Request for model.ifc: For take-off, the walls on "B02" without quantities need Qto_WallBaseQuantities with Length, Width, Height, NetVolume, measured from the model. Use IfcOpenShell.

First a look at what the model holds.

```python
import ifcopenshell
import ifcopenshell.util.element
import ifcopenshell.util.unit

model = ifcopenshell.open("model.ifc")
print(model.schema)
for unit_type in ("LENGTHUNIT", "AREAUNIT", "VOLUMEUNIT"):
    print(unit_type, ifcopenshell.util.unit.calculate_unit_scale(model, unit_type))
storey = next(s for s in model.by_type("IfcBuildingStorey") if s.Name == "B02")
walls = [e for e in ifcopenshell.util.element.get_decomposition(storey) if e.is_a("IfcWall")]
for e in sorted(walls, key=lambda e: e.id()):
    print(e.id(), e.is_a(), e.Name, list(ifcopenshell.util.element.get_psets(e, qtos_only=True)), sep=" | ")
```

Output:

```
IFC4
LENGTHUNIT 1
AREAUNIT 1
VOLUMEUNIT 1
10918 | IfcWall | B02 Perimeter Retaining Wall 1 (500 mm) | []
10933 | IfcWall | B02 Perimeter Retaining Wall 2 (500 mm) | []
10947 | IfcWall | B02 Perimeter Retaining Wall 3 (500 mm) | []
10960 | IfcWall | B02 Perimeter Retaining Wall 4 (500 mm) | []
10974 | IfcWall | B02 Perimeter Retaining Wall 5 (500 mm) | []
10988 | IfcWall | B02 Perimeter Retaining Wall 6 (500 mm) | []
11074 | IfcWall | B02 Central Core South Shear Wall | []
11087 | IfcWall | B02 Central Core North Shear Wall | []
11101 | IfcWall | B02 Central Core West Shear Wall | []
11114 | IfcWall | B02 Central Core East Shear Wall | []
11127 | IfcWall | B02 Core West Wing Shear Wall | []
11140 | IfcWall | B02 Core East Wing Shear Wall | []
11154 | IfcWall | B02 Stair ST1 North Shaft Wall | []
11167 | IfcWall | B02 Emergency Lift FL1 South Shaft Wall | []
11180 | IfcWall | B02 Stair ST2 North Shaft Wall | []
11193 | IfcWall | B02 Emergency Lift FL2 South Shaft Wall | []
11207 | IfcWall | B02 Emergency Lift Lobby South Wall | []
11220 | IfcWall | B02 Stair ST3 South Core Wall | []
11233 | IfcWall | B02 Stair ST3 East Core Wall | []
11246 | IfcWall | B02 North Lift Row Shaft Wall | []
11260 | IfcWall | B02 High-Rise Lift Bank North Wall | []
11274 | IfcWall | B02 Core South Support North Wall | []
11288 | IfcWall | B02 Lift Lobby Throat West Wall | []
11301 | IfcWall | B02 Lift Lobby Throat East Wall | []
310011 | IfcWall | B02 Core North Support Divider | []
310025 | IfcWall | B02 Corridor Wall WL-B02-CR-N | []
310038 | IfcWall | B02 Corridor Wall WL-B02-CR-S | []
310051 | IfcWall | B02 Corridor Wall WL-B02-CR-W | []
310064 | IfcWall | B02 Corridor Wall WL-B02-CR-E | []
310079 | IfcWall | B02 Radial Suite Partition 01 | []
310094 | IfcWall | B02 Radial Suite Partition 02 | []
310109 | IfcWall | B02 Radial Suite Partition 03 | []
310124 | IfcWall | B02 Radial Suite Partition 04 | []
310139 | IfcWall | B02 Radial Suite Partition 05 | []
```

```python
import ifcopenshell
import ifcopenshell.api.pset
import ifcopenshell.geom
import ifcopenshell.util.element
import ifcopenshell.util.shape
import ifcopenshell.util.unit

model = ifcopenshell.open("model.ifc")
unit_scale = ifcopenshell.util.unit.calculate_unit_scale(model)
volume_scale = ifcopenshell.util.unit.calculate_unit_scale(model, "VOLUMEUNIT")
settings = ifcopenshell.geom.settings()

storey = next(s for s in model.by_type("IfcBuildingStorey") if s.Name == "B02")
walls = [e for e in ifcopenshell.util.element.get_decomposition(storey) if e.is_a("IfcWall")]

for e in sorted(walls, key=lambda e: e.id()):
    if ifcopenshell.util.element.get_psets(e, qtos_only=True, should_inherit=False):
        continue
    # Geometry comes back in metres, in the element's own axes.
    shape = ifcopenshell.geom.create_shape(settings, e)
    values = {
        "Length": ifcopenshell.util.shape.get_x(shape.geometry) / unit_scale,
        "Width": ifcopenshell.util.shape.get_y(shape.geometry) / unit_scale,
        "Height": ifcopenshell.util.shape.get_z(shape.geometry) / unit_scale,
        "NetVolume": ifcopenshell.util.shape.get_volume(shape.geometry) / volume_scale,
    }
    qto = ifcopenshell.api.pset.add_qto(model, product=e, name="Qto_WallBaseQuantities")
    ifcopenshell.api.pset.edit_qto(model, qto=qto, properties=values)
    print(e.id(), {k: round(v, 3) for k, v in values.items()})

model.write("model_rev.ifc")
```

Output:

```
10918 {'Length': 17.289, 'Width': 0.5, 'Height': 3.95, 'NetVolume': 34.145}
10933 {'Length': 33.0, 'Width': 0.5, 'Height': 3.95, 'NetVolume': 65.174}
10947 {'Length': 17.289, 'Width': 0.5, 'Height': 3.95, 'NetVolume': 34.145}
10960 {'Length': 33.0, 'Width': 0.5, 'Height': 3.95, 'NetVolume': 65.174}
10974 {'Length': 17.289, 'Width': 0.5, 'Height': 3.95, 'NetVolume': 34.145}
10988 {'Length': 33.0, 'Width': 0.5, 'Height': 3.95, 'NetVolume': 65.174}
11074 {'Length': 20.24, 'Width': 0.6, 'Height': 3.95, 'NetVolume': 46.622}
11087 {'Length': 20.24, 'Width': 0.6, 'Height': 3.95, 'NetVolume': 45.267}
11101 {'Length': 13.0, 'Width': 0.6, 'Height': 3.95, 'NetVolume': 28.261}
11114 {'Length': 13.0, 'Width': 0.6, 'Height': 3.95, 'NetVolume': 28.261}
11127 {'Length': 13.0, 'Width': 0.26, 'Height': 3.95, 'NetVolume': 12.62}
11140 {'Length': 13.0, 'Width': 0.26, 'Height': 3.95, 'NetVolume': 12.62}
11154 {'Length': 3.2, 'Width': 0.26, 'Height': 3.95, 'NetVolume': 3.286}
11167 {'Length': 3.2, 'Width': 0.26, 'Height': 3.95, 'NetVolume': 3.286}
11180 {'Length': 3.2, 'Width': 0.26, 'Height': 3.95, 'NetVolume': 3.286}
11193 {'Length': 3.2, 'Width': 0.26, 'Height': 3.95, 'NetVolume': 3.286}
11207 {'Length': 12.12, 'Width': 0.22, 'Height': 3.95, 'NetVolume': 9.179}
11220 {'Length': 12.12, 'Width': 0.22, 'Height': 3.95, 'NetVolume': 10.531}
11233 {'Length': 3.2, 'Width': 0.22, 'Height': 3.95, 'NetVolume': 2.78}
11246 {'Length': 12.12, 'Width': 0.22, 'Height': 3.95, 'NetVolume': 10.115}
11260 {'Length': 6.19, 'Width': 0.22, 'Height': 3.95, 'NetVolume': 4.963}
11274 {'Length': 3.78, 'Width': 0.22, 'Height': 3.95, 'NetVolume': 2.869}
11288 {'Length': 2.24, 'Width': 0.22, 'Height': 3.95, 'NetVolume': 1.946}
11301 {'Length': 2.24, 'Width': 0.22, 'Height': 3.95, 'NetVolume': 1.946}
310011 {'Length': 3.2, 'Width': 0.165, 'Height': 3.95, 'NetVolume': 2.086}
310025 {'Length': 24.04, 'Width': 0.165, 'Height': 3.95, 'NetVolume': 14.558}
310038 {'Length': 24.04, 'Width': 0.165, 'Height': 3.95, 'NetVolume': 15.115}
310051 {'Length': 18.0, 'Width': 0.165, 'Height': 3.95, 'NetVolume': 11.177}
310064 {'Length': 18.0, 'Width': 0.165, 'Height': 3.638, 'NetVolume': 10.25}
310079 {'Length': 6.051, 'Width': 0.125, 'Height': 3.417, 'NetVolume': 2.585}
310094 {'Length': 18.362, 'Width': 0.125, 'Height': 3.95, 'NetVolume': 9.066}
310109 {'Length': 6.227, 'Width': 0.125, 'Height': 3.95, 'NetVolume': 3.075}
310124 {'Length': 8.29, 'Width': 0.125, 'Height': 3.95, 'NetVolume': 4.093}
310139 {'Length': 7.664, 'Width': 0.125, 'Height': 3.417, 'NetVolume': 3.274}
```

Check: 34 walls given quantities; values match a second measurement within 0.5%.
